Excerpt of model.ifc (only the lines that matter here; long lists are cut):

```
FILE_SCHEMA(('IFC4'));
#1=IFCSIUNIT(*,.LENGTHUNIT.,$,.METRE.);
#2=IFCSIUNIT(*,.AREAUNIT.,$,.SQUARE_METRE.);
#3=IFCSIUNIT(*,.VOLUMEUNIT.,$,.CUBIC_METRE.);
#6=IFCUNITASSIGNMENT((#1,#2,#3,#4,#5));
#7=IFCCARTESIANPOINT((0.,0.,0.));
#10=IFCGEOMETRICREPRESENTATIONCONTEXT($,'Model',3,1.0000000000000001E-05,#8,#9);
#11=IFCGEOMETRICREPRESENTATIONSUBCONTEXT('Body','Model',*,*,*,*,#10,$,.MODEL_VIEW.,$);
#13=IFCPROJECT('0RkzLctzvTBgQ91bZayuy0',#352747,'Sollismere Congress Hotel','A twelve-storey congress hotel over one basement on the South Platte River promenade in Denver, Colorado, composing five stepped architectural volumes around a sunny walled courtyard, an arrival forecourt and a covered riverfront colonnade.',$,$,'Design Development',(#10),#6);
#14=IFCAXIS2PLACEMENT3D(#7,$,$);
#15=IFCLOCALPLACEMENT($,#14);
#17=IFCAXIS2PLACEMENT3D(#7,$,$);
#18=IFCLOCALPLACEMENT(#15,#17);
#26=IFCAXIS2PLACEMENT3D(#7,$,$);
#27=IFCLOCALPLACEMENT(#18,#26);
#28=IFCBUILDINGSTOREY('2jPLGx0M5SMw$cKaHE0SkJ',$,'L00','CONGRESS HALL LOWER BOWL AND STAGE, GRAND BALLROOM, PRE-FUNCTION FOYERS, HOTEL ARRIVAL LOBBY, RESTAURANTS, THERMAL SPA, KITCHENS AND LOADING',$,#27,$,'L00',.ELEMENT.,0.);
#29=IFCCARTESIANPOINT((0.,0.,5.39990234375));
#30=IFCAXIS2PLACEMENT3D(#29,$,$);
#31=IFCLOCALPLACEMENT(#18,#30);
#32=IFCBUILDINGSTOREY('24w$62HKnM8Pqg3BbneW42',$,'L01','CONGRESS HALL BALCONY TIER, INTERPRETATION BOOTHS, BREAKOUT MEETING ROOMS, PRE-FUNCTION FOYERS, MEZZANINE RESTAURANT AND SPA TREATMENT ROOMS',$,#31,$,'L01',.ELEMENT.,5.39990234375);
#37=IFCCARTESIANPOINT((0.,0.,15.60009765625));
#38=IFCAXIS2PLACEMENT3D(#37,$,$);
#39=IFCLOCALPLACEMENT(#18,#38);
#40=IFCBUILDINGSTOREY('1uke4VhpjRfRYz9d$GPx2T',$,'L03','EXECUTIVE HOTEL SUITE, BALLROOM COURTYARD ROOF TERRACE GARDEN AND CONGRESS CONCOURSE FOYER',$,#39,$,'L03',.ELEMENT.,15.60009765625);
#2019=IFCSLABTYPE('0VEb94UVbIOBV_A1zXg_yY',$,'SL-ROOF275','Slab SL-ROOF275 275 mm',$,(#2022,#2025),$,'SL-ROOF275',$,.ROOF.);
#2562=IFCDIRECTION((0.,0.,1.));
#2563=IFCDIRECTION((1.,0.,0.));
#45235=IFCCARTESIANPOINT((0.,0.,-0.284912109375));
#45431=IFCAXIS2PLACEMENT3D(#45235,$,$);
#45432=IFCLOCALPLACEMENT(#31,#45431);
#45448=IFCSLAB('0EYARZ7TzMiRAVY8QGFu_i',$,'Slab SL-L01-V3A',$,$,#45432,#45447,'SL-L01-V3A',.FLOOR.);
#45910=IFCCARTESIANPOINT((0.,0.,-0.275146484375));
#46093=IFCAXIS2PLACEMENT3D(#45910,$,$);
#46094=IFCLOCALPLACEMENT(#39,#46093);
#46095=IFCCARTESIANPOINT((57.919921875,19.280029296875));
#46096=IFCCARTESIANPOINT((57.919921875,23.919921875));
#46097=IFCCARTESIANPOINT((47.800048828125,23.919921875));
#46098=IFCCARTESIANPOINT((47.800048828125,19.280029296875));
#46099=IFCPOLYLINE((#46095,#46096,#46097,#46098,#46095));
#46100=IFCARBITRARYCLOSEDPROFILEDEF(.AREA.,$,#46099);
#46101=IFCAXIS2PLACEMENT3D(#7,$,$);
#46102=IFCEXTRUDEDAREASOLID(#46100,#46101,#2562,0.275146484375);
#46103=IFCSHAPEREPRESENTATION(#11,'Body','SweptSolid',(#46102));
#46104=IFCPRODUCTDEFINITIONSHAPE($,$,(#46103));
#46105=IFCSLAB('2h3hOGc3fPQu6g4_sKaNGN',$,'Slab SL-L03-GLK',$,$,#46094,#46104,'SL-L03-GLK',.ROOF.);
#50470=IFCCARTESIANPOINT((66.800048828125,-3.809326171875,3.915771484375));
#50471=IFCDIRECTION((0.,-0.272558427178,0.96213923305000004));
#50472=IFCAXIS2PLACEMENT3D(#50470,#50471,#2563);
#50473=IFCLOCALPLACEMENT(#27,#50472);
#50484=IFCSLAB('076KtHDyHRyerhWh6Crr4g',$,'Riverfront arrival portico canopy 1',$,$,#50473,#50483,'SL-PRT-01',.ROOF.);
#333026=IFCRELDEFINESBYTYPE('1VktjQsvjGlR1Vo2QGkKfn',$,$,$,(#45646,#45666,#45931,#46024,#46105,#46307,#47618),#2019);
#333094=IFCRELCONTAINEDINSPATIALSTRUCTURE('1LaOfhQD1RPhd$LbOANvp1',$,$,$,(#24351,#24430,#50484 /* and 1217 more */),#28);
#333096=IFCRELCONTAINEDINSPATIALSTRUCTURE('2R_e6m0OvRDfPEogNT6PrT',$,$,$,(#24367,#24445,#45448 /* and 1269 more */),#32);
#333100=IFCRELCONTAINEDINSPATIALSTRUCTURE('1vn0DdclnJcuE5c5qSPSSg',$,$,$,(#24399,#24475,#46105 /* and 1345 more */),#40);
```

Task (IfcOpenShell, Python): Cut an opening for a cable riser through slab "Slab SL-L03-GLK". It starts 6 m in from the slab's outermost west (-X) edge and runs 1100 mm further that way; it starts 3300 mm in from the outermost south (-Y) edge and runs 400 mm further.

```python
import numpy as np
import ifcopenshell
import ifcopenshell.api.feature
import ifcopenshell.api.geometry
import ifcopenshell.api.root
import ifcopenshell.geom
import ifcopenshell.util.placement
import ifcopenshell.util.representation
import ifcopenshell.util.shape
import ifcopenshell.util.unit

model = ifcopenshell.open("model.ifc")
unit_scale = ifcopenshell.util.unit.calculate_unit_scale(model)
settings = ifcopenshell.geom.settings()


def volume(element):
    """Net volume in cubic metres, openings subtracted."""
    shape = ifcopenshell.geom.create_shape(settings, element)
    return ifcopenshell.util.shape.get_volume(shape.geometry)


slab = model.by_id(46105)
before = volume(slab)

# Extent in the slab's own axes, in metres. The edges named are its -X and -Y sides.
slab_shape = ifcopenshell.geom.create_shape(settings, slab)
vertices = ifcopenshell.util.shape.get_vertices(slab_shape.geometry)
x_min, y_min, bottom = vertices.min(axis=0)
top = vertices[:, 2].max()

opening = ifcopenshell.api.root.create_entity(model, ifc_class="IfcOpeningElement", name="Cable riser opening", predefined_type="OPENING")
context = ifcopenshell.util.representation.get_context(model, "Model", "Body", "MODEL_VIEW")
width, depth = 1.1, 0.4
outline = [(0.0, 0.0), (width, 0.0), (width, depth), (0.0, depth), (0.0, 0.0)]
# Overshoot both faces by 50 mm so the cut is clean.
shape = ifcopenshell.api.geometry.add_slab_representation(
    model, context=context, depth=top - bottom + 0.1, polyline=outline
)
ifcopenshell.api.geometry.assign_representation(model, product=opening, representation=shape)

matrix = ifcopenshell.util.placement.get_local_placement(slab.ObjectPlacement)
matrix[:, 3] = matrix @ np.append(np.array([x_min + 6, y_min + 3.3, bottom - 0.05]) / unit_scale, 1.0)
ifcopenshell.api.geometry.edit_object_placement(model, product=opening, matrix=matrix, is_si=False)
ifcopenshell.api.feature.add_feature(model, feature=opening, element=slab)

after = volume(slab)

print(f"slab volume {before:.3f} -> {after:.3f} m3")

model.write("model_v2.ifc")
```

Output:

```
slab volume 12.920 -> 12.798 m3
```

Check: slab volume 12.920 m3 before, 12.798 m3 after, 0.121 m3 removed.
